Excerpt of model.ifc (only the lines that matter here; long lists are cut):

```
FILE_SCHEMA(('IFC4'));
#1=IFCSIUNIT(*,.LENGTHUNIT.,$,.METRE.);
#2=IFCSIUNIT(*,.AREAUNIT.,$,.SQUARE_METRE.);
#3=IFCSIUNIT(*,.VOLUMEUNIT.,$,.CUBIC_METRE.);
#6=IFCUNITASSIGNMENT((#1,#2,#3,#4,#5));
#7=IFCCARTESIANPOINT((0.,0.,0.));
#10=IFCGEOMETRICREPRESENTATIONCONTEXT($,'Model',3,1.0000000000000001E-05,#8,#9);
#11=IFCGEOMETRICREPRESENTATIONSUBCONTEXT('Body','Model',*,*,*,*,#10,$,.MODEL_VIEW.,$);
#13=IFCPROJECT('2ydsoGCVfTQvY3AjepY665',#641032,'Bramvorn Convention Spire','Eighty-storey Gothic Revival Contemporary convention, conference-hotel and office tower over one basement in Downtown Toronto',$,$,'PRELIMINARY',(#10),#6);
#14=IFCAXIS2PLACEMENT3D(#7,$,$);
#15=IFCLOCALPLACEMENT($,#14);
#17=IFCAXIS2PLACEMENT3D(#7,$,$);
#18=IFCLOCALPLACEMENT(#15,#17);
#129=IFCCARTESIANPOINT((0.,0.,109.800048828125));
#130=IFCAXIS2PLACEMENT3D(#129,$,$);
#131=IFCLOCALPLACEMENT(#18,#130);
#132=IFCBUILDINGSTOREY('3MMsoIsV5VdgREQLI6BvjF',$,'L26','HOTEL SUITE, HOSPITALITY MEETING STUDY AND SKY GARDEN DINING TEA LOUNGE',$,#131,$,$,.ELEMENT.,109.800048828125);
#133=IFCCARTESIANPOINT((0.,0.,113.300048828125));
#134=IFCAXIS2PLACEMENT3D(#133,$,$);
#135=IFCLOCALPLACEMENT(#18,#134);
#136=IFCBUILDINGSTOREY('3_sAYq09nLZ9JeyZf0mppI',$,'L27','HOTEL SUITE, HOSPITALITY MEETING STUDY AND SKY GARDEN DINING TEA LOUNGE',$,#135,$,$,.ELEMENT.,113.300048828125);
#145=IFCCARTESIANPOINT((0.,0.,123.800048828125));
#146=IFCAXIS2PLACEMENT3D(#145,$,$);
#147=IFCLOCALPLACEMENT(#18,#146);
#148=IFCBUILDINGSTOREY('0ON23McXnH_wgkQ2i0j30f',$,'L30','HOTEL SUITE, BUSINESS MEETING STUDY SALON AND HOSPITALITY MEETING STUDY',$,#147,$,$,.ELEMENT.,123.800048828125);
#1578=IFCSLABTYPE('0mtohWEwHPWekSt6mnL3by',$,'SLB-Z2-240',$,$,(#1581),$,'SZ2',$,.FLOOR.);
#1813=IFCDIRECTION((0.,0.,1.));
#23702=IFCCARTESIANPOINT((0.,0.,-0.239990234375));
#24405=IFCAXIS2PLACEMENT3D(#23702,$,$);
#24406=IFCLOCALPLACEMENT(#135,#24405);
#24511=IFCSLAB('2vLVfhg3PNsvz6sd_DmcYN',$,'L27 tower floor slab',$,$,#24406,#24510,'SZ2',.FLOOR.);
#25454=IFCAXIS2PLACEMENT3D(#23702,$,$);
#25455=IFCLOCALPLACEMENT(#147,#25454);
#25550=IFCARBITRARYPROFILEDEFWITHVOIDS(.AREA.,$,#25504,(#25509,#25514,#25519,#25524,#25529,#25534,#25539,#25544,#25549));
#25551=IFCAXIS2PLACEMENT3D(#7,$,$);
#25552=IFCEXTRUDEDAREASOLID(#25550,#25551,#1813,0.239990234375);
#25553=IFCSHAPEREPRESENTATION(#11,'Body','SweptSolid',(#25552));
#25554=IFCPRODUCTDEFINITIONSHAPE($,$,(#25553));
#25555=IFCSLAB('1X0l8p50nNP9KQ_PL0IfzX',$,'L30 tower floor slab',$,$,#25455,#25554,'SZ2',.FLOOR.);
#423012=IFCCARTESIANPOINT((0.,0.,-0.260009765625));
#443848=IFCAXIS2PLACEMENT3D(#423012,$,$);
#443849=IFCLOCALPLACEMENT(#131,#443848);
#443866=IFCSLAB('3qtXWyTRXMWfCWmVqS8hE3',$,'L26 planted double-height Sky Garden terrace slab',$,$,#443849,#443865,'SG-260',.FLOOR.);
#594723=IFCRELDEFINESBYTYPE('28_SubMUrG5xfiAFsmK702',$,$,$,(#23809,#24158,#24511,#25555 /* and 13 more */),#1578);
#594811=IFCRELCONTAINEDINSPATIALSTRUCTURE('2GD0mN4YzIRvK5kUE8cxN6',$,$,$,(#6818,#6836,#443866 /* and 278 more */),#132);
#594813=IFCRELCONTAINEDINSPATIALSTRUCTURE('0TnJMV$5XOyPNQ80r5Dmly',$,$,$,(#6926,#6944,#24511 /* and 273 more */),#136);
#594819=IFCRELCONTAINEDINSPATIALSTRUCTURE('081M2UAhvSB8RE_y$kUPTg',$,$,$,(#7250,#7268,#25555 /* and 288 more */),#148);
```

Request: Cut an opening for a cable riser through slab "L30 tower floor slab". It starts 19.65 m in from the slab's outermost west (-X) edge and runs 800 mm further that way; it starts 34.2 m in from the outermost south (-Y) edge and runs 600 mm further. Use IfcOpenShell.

```python
import numpy as np
import ifcopenshell
import ifcopenshell.api.feature
import ifcopenshell.api.geometry
import ifcopenshell.api.root
import ifcopenshell.geom
import ifcopenshell.util.placement
import ifcopenshell.util.representation
import ifcopenshell.util.shape
import ifcopenshell.util.unit

model = ifcopenshell.open("model.ifc")
unit_scale = ifcopenshell.util.unit.calculate_unit_scale(model)
settings = ifcopenshell.geom.settings()


def volume(element):
    """Net volume in cubic metres, openings subtracted."""
    shape = ifcopenshell.geom.create_shape(settings, element)
    return ifcopenshell.util.shape.get_volume(shape.geometry)


slab = model.by_id(25555)
before = volume(slab)

# Extent in the slab's own axes, in metres. The edges named are its -X and -Y sides.
slab_shape = ifcopenshell.geom.create_shape(settings, slab)
vertices = ifcopenshell.util.shape.get_vertices(slab_shape.geometry)
x_min, y_min, bottom = vertices.min(axis=0)
top = vertices[:, 2].max()

opening = ifcopenshell.api.root.create_entity(model, ifc_class="IfcOpeningElement", name="Cable riser opening", predefined_type="OPENING")
context = ifcopenshell.util.representation.get_context(model, "Model", "Body", "MODEL_VIEW")
width, depth = 0.8, 0.6
outline = [(0.0, 0.0), (width, 0.0), (width, depth), (0.0, depth), (0.0, 0.0)]
# Overshoot both faces by 50 mm so the cut is clean.
shape = ifcopenshell.api.geometry.add_slab_representation(
    model, context=context, depth=top - bottom + 0.1, polyline=outline
)
ifcopenshell.api.geometry.assign_representation(model, product=opening, representation=shape)

matrix = ifcopenshell.util.placement.get_local_placement(slab.ObjectPlacement)
matrix[:, 3] = matrix @ np.append(np.array([x_min + 19.65, y_min + 34.2, bottom - 0.05]) / unit_scale, 1.0)
ifcopenshell.api.geometry.edit_object_placement(model, product=opening, matrix=matrix, is_si=False)
ifcopenshell.api.feature.add_feature(model, feature=opening, element=slab)

after = volume(slab)

print(f"slab volume {before:.3f} -> {after:.3f} m3")

model.write("model_rev.ifc")
```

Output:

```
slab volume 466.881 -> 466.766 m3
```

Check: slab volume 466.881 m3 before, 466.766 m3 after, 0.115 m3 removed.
